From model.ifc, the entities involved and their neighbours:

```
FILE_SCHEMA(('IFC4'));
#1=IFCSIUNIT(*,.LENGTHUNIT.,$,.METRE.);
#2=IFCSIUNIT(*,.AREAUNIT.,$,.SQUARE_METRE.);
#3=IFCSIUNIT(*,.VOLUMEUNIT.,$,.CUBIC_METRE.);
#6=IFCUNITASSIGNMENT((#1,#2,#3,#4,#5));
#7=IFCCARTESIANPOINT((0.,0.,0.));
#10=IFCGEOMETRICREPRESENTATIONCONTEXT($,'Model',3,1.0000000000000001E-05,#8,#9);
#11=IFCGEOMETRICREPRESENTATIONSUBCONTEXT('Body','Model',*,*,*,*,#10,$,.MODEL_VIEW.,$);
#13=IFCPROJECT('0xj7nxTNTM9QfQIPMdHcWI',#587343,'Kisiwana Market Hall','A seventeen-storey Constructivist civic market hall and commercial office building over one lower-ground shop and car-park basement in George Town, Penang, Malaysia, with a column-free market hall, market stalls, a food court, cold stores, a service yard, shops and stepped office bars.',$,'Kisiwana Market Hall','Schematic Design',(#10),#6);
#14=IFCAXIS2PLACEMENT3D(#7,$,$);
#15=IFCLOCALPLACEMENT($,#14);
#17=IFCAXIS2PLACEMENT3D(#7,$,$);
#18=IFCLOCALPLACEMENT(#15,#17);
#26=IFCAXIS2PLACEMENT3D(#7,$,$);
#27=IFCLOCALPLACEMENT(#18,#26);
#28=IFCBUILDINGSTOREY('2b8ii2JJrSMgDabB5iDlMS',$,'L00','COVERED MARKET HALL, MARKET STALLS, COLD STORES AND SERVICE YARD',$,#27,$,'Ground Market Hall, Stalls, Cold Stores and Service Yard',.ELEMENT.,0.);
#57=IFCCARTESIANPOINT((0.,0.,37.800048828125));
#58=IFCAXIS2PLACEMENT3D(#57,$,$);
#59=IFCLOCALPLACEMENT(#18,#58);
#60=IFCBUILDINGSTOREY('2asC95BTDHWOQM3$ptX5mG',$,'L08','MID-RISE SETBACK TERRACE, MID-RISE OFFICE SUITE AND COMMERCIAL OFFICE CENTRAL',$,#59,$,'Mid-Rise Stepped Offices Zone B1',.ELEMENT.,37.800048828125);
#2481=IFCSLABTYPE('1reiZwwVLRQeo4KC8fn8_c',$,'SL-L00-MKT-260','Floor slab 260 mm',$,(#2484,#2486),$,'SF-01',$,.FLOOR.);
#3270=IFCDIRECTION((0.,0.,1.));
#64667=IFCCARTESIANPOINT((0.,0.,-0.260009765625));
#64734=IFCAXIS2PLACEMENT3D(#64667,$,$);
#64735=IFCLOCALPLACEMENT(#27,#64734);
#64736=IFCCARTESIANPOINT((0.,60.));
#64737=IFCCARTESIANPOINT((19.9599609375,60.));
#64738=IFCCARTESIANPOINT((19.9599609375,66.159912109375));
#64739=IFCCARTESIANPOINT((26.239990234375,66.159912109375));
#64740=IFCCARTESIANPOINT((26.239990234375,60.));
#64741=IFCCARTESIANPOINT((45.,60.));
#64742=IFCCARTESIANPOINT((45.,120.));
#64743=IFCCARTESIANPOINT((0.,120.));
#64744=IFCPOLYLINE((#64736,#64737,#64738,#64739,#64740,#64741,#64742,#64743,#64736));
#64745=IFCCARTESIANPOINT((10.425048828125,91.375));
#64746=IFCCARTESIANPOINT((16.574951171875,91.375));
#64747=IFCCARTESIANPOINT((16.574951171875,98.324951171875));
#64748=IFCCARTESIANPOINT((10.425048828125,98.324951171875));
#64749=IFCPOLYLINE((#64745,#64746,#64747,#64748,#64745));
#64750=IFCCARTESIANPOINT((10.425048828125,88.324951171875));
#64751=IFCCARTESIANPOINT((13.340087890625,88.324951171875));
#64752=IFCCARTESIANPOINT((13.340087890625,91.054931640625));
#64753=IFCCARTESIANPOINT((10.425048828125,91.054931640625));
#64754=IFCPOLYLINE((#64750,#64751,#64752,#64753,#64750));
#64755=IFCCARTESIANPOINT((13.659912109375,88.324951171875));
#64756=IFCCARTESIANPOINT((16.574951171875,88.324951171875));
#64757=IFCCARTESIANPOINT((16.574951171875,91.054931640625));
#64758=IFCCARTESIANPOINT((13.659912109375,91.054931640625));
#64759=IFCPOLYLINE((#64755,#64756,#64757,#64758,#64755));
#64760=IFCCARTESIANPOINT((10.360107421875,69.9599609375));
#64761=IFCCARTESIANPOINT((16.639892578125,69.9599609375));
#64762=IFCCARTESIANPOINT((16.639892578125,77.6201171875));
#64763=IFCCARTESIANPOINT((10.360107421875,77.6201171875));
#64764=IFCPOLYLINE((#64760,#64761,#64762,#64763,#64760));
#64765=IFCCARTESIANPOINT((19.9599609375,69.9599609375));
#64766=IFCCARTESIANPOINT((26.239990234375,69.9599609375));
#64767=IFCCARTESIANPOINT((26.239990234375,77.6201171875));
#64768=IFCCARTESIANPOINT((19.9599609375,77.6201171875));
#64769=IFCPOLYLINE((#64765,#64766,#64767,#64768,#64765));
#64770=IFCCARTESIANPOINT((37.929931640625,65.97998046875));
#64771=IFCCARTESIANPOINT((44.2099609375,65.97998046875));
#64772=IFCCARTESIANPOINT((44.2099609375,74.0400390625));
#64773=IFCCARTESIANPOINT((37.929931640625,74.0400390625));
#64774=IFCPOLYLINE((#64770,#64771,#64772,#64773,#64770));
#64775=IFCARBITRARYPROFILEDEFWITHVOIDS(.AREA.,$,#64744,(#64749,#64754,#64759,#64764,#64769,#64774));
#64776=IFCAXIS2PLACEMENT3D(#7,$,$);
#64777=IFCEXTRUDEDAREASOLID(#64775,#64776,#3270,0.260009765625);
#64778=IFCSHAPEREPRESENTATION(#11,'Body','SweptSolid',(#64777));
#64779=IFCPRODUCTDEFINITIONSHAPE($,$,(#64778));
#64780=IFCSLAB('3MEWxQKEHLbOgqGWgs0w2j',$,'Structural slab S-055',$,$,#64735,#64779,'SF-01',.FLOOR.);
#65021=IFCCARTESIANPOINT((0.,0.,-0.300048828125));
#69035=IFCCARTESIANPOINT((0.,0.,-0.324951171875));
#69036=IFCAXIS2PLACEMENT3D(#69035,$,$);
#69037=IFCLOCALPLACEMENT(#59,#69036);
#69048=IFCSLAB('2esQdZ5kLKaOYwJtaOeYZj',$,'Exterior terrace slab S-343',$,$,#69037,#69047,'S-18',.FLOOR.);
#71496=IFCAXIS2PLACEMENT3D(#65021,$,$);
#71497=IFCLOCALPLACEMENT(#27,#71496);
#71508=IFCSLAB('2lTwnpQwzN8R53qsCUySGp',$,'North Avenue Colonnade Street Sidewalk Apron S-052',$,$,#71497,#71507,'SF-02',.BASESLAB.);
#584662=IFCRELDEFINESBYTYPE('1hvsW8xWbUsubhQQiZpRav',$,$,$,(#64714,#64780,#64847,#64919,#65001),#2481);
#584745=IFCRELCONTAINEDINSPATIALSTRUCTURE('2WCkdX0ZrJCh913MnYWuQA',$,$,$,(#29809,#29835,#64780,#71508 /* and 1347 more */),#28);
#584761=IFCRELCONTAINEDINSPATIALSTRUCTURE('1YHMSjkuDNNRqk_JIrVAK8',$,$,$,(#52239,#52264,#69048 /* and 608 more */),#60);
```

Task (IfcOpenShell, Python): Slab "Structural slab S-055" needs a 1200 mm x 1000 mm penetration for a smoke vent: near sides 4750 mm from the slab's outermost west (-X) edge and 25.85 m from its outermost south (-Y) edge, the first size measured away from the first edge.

```python
import numpy as np
import ifcopenshell
import ifcopenshell.api.feature
import ifcopenshell.api.geometry
import ifcopenshell.api.root
import ifcopenshell.geom
import ifcopenshell.util.placement
import ifcopenshell.util.representation
import ifcopenshell.util.shape
import ifcopenshell.util.unit

model = ifcopenshell.open("model.ifc")
unit_scale = ifcopenshell.util.unit.calculate_unit_scale(model)
settings = ifcopenshell.geom.settings()


def volume(element):
    """Net volume in cubic metres, openings subtracted."""
    shape = ifcopenshell.geom.create_shape(settings, element)
    return ifcopenshell.util.shape.get_volume(shape.geometry)


slab = model.by_guid("3MEWxQKEHLbOgqGWgs0w2j")
before = volume(slab)

# Extent in the slab's own axes, in metres. The edges named are its -X and -Y sides.
slab_shape = ifcopenshell.geom.create_shape(settings, slab)
vertices = ifcopenshell.util.shape.get_vertices(slab_shape.geometry)
x_min, y_min, bottom = vertices.min(axis=0)
top = vertices[:, 2].max()

opening = ifcopenshell.api.root.create_entity(model, ifc_class="IfcOpeningElement", name="Smoke vent opening", predefined_type="OPENING")
context = ifcopenshell.util.representation.get_context(model, "Model", "Body", "MODEL_VIEW")
width, depth = 1.2, 1
outline = [(0.0, 0.0), (width, 0.0), (width, depth), (0.0, depth), (0.0, 0.0)]
# Overshoot both faces by 50 mm so the cut is clean.
shape = ifcopenshell.api.geometry.add_slab_representation(
    model, context=context, depth=top - bottom + 0.1, polyline=outline
)
ifcopenshell.api.geometry.assign_representation(model, product=opening, representation=shape)

matrix = ifcopenshell.util.placement.get_local_placement(slab.ObjectPlacement)
matrix[:, 3] = matrix @ np.append(np.array([x_min + 4.75, y_min + 25.85, bottom - 0.05]) / unit_scale, 1.0)
ifcopenshell.api.geometry.edit_object_placement(model, product=opening, matrix=matrix, is_si=False)
ifcopenshell.api.feature.add_feature(model, feature=opening, element=slab)

after = volume(slab)

print(f"slab volume {before:.3f} -> {after:.3f} m3")

model.write("model_updated.ifc")
```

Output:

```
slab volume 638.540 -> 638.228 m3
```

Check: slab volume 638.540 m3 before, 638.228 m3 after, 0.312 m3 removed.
